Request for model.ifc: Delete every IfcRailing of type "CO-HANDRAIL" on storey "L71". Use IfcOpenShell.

First a look at what the model holds.

```python
import ifcopenshell
import ifcopenshell.util.element

model = ifcopenshell.open("model.ifc")
print(model.schema)
storey = next(s for s in model.by_type("IfcBuildingStorey") if s.Name == "L71")
railings = [e for e in ifcopenshell.util.element.get_decomposition(storey) if e.is_a("IfcRailing")]
seen = {}
for e in railings:
    element_type = ifcopenshell.util.element.get_type(e)
    name = element_type.Name if element_type not in (None, e) else None
    seen[name] = seen.get(name, 0) + 1
for name, count in sorted(seen.items(), key=str):
    print(count, "x", name)
```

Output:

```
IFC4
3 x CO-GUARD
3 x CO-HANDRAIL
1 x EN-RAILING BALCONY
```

```python
import ifcopenshell
import ifcopenshell.api.root
import ifcopenshell.util.element

model = ifcopenshell.open("model.ifc")

storey = next(s for s in model.by_type("IfcBuildingStorey") if s.Name == "L71")
railings = [e for e in ifcopenshell.util.element.get_decomposition(storey) if e.is_a("IfcRailing")]
targets = [e for e in railings if (t := ifcopenshell.util.element.get_type(e)) not in (None, e) and t.Name == "CO-HANDRAIL"]

for e in targets:
    ifcopenshell.api.root.remove_product(model, product=e)
print(len(targets), "removed")

model.write("model_edited.ifc")
```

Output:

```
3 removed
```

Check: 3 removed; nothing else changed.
